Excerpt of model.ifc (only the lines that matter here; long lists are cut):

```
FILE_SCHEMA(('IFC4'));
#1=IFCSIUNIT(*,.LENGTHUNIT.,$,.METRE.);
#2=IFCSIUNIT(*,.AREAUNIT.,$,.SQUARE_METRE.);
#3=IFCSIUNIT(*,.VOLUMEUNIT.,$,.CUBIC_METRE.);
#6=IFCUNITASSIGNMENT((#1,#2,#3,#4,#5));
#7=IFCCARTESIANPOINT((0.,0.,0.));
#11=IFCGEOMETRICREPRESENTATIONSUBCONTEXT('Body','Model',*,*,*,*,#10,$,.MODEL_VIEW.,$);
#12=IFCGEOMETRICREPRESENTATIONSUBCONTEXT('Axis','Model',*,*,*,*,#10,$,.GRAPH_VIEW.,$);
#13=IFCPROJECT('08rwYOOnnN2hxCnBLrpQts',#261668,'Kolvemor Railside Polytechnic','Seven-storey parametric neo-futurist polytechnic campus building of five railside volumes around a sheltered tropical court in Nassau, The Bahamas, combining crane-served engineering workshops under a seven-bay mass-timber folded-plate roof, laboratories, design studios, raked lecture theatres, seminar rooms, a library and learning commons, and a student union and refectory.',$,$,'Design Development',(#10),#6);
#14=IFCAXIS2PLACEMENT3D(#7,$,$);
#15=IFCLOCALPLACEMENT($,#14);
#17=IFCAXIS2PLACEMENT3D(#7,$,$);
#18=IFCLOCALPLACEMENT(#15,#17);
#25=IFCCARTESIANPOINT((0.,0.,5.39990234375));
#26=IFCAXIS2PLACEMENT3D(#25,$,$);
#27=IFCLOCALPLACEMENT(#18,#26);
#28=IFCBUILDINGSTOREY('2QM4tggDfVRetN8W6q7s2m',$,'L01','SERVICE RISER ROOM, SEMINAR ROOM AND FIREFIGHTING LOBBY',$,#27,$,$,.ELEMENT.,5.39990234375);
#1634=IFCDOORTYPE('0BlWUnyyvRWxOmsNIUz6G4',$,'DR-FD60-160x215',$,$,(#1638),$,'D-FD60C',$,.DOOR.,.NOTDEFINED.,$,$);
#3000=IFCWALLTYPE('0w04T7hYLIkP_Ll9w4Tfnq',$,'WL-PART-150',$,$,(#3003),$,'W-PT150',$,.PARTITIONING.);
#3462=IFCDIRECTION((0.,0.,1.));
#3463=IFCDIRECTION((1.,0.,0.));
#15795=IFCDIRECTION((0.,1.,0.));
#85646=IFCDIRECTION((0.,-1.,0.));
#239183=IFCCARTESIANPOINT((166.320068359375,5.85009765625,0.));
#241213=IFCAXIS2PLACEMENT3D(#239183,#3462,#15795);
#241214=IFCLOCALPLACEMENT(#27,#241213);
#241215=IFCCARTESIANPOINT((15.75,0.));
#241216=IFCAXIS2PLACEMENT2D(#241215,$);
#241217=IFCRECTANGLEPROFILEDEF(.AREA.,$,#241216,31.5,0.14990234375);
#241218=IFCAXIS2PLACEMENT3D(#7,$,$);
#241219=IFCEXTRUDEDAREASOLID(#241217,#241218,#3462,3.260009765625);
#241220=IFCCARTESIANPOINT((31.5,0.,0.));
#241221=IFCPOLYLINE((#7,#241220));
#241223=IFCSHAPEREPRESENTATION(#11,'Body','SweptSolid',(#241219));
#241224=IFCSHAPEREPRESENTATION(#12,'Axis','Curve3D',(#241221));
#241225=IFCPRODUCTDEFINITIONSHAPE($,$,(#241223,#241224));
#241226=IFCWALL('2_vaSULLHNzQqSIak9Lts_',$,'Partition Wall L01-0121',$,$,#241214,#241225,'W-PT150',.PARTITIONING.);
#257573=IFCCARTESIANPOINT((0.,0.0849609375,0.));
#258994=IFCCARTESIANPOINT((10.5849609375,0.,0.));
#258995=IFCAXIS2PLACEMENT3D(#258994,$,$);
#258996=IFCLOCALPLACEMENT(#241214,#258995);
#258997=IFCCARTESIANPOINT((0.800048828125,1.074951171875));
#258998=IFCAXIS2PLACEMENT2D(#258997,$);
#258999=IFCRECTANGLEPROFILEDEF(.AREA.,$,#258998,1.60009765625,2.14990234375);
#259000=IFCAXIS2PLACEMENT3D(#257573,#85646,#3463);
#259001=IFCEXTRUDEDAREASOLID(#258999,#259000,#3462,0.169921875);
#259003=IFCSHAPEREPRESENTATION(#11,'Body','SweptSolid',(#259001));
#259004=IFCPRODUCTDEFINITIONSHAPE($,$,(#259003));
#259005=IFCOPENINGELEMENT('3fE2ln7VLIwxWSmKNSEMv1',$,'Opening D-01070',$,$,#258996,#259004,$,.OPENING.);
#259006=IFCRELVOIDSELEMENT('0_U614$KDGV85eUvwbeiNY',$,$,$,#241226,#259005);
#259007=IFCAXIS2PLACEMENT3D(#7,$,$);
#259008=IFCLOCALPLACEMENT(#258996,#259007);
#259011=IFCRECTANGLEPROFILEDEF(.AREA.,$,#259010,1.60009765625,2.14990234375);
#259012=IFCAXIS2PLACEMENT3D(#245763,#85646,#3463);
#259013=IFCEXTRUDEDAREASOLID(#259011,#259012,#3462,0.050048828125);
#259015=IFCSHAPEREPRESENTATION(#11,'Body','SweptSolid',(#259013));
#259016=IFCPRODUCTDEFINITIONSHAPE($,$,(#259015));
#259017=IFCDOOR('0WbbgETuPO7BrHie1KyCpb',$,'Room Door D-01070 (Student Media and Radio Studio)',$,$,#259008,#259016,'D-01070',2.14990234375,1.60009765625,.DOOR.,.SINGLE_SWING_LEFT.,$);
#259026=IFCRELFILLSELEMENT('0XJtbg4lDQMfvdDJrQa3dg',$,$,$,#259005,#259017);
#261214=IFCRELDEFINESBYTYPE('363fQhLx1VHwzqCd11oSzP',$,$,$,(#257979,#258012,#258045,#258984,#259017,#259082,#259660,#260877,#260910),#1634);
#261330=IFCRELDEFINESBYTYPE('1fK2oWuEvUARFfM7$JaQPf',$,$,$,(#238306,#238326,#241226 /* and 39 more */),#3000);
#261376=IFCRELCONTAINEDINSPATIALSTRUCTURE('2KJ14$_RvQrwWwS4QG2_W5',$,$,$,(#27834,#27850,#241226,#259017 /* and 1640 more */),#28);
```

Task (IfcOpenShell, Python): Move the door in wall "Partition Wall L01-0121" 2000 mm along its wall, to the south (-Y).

```python
import ifcopenshell
import ifcopenshell.api.geometry
import ifcopenshell.util.placement

model = ifcopenshell.open("model.ifc")

door = model.by_id(259017)
opening = door.FillsVoids[0].RelatingOpeningElement
wall = opening.VoidsElements[0].RelatingBuildingElement

wall_matrix = ifcopenshell.util.placement.get_local_placement(wall.ObjectPlacement)
shift = wall_matrix[:3, 0] * -2.0
before = ifcopenshell.util.placement.get_local_placement(door.ObjectPlacement)[:3, 3].copy()

# The door is placed relative to its opening, so it follows when the opening moves.
matrix = ifcopenshell.util.placement.get_local_placement(opening.ObjectPlacement)
matrix[:3, 3] += shift
ifcopenshell.api.geometry.edit_object_placement(
    model, product=opening, matrix=matrix, is_si=False, should_transform_children=True
)

after = ifcopenshell.util.placement.get_local_placement(door.ObjectPlacement)[:3, 3]
print("door moved by", (after - before).round(3) + 0.0)

model.write("model_edited.ifc")
```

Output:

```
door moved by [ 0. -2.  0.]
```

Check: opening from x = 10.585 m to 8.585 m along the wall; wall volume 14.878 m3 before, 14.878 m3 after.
